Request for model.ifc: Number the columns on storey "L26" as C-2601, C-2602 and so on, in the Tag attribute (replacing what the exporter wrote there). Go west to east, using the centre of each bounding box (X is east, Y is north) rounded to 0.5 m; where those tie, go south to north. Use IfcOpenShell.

First a look at what the model holds.

```python
import ifcopenshell
import ifcopenshell.util.element
import ifcopenshell.util.placement

model = ifcopenshell.open("model.ifc")
print(model.schema)
storey = next(s for s in model.by_type("IfcBuildingStorey") if s.Name == "L26")
columns = [e for e in ifcopenshell.util.element.get_decomposition(storey) if e.is_a("IfcColumn")]
for e in sorted(columns, key=lambda e: e.id()):
    origin = ifcopenshell.util.placement.get_local_placement(e.ObjectPlacement)[:3, 3]
    print(e.id(), e.Tag, e.Name, origin.round(2) + 0.0, sep=" | ")
```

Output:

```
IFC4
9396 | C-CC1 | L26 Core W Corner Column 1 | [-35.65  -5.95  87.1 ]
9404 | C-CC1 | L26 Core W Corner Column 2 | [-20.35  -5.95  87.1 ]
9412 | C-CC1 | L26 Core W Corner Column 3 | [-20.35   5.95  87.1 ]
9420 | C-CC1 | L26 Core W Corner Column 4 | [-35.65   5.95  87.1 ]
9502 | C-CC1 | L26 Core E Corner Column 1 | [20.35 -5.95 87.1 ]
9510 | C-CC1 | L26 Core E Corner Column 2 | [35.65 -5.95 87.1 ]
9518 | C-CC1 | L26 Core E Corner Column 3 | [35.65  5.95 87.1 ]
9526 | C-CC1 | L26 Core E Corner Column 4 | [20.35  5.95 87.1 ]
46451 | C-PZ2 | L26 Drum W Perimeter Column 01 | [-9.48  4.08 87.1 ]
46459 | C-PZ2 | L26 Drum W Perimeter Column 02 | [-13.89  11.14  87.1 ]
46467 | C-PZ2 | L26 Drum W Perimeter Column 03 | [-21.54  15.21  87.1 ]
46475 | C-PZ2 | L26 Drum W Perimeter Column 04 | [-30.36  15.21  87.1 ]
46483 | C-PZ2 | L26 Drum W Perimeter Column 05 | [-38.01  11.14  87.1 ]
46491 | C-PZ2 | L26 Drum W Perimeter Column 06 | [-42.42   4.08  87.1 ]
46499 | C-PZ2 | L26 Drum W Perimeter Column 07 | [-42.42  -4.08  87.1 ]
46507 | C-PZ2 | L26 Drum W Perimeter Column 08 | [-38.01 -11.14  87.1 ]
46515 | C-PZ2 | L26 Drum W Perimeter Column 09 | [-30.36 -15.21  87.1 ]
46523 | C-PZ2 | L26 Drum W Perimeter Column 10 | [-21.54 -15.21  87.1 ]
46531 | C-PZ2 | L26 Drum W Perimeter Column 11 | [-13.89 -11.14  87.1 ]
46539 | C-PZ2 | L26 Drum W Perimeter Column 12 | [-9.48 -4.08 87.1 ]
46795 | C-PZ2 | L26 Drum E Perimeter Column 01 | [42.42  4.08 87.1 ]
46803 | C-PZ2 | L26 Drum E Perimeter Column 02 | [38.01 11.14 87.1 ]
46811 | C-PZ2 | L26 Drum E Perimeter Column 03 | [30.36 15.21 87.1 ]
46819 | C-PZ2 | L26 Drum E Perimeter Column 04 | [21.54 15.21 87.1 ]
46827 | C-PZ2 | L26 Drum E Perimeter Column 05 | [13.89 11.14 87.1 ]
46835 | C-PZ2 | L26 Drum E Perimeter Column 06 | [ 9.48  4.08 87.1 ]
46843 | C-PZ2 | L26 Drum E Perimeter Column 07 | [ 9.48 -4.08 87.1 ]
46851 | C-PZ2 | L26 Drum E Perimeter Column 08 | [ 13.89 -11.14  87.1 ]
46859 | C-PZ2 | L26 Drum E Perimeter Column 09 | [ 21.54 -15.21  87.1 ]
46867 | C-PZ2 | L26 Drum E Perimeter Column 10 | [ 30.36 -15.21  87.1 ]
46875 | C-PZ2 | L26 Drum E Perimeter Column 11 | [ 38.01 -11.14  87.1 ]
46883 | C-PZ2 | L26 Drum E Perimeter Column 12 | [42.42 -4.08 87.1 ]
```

```python
import ifcopenshell
import ifcopenshell.geom
import ifcopenshell.util.element
import ifcopenshell.util.shape

model = ifcopenshell.open("model.ifc")
settings = ifcopenshell.geom.settings()
settings.set("use-world-coords", True)


def centre(element):
    shape = ifcopenshell.geom.create_shape(settings, element)
    return ifcopenshell.util.shape.get_bbox_centroid(shape.geometry)


storey = next(s for s in model.by_type("IfcBuildingStorey") if s.Name == "L26")
columns = [e for e in ifcopenshell.util.element.get_decomposition(storey) if e.is_a("IfcColumn")]

# Insertion points can sit at a corner or the storey origin, so sort by the geometry (in metres).
centres = {e: centre(e) for e in columns}
columns.sort(key=lambda e: (round(centres[e][0] / 0.5), centres[e][1]))

for i, e in enumerate(columns, start=1):
    number = f"C-26{i:02d}"
    e.Tag = number
    print(e.id(), number)

model.write("model_rev.ifc")
```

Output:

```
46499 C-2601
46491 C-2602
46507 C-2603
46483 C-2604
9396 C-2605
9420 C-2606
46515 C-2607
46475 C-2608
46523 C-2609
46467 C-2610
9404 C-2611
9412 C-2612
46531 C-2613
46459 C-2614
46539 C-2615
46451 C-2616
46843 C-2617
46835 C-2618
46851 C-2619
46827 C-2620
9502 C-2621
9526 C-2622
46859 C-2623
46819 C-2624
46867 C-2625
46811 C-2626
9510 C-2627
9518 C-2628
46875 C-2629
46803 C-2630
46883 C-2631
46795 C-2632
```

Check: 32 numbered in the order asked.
